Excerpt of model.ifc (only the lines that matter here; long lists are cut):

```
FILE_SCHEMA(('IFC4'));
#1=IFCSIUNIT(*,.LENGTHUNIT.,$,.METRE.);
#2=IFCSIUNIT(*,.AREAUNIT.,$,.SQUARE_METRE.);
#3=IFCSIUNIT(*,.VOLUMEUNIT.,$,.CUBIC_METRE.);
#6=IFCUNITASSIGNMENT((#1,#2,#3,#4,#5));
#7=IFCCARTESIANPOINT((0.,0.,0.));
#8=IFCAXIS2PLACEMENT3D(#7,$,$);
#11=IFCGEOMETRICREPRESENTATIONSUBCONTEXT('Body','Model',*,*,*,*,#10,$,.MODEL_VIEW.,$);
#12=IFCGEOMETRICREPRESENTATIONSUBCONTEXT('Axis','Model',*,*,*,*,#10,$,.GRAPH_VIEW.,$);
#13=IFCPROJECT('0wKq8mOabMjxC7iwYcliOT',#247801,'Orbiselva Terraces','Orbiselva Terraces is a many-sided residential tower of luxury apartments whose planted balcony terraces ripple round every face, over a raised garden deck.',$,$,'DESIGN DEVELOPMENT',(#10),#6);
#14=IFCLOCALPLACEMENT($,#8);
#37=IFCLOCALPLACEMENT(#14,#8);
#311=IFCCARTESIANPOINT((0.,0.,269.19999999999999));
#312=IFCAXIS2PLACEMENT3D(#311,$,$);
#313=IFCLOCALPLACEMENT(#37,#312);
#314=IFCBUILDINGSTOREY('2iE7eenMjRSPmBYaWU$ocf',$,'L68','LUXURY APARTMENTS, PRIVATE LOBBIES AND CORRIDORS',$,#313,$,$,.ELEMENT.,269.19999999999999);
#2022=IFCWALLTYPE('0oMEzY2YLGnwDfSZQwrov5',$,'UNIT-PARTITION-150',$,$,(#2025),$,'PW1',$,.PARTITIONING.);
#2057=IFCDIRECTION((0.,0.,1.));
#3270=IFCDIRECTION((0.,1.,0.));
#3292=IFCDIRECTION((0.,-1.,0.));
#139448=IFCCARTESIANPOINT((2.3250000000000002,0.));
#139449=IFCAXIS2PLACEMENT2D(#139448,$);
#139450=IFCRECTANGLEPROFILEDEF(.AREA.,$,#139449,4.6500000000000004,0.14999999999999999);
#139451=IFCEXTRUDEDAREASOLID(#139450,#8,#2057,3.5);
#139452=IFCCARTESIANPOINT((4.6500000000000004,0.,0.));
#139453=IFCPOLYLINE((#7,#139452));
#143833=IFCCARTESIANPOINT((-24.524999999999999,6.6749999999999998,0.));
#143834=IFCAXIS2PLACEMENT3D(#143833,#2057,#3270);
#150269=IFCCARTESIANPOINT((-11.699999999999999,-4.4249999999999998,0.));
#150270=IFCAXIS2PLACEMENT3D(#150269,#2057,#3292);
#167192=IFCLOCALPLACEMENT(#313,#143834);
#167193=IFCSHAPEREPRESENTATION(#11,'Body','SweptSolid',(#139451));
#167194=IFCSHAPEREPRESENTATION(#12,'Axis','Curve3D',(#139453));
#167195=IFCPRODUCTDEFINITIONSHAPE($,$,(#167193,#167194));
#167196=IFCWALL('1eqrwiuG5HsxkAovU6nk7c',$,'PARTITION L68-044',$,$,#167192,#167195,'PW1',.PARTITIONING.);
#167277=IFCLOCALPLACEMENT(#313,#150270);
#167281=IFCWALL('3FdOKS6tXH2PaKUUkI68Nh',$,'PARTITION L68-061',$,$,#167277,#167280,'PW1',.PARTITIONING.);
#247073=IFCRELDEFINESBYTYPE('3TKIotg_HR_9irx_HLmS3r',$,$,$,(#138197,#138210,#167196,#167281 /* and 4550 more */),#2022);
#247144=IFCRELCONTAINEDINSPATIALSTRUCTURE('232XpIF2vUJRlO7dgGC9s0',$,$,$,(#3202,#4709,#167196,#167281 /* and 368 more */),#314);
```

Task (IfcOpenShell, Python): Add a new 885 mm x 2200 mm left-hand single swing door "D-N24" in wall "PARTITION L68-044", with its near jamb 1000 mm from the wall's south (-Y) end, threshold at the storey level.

```python
import numpy as np
import ifcopenshell
import ifcopenshell.api.feature
import ifcopenshell.api.geometry
import ifcopenshell.api.root
import ifcopenshell.api.spatial
import ifcopenshell.geom
import ifcopenshell.util.element
import ifcopenshell.util.placement
import ifcopenshell.util.representation
import ifcopenshell.util.shape
import ifcopenshell.util.unit

model = ifcopenshell.open("model.ifc")
unit_scale = ifcopenshell.util.unit.calculate_unit_scale(model)
settings = ifcopenshell.geom.settings()


def volume(element):
    """Net volume in cubic metres, openings subtracted."""
    shape = ifcopenshell.geom.create_shape(settings, element)
    return ifcopenshell.util.shape.get_volume(shape.geometry)


wall = model.by_guid("1eqrwiuG5HsxkAovU6nk7c")
storey = ifcopenshell.util.element.get_container(wall, ifc_class="IfcBuildingStorey")
context = ifcopenshell.util.representation.get_context(model, "Model", "Body", "MODEL_VIEW")
before = volume(wall)

width, height, from_end, sill = 0.885, 2.2, 1, 0.0  # metres

# The wall runs along its own X axis, and the end named is its -X end.
wall_shape = ifcopenshell.geom.create_shape(settings, wall)
x, y, z = ifcopenshell.util.shape.get_vertices(wall_shape.geometry).T
start = x.min() + from_end
face, thickness = float(y.min()), float(y.max() - y.min())
wall_matrix = ifcopenshell.util.placement.get_local_placement(wall.ObjectPlacement)
level = ifcopenshell.util.placement.get_local_placement(storey.ObjectPlacement)[2, 3]


def in_wall(x, y):
    """Placement at x, y metres in the wall's axes, at sill height."""
    matrix = wall_matrix.copy()
    matrix[:, 3] = wall_matrix @ np.array([x / unit_scale, y / unit_scale, 0.0, 1.0])
    matrix[2, 3] = level + sill / unit_scale
    return matrix


# Opening: a box that overshoots both wall faces by 50 mm.
opening = ifcopenshell.api.root.create_entity(model, ifc_class="IfcOpeningElement", predefined_type="OPENING")
box = ifcopenshell.api.geometry.add_wall_representation(
    model, context=context, length=width, height=height, thickness=thickness + 0.1
)
ifcopenshell.api.geometry.assign_representation(model, product=opening, representation=box)
ifcopenshell.api.geometry.edit_object_placement(model, product=opening, matrix=in_wall(start, face - 0.05), is_si=False)
ifcopenshell.api.feature.add_feature(model, feature=opening, element=wall)

door = ifcopenshell.api.root.create_entity(model, ifc_class="IfcDoor", name="D-N24", predefined_type="DOOR")
door.OverallWidth, door.OverallHeight = width / unit_scale, height / unit_scale
door.OperationType = "SINGLE_SWING_LEFT"
body = ifcopenshell.api.geometry.add_door_representation(
    model,
    context=context,
    overall_width=door.OverallWidth,
    overall_height=door.OverallHeight,
    operation_type="SINGLE_SWING_LEFT",
    lining_properties={"LiningDepth": thickness / unit_scale, "ThresholdDepth": thickness / unit_scale},
)
ifcopenshell.api.geometry.assign_representation(model, product=door, representation=body)
ifcopenshell.api.spatial.assign_container(model, products=[door], relating_structure=storey)
ifcopenshell.api.feature.add_filling(model, opening=opening, element=door)

# The lining spans the wall, so the door starts at the wall face.
ifcopenshell.api.geometry.edit_object_placement(model, product=door, matrix=in_wall(start, face), is_si=False)

after = volume(wall)

print(f"wall volume {before:.3f} -> {after:.3f} m3")

model.write("model_v2.ifc")
```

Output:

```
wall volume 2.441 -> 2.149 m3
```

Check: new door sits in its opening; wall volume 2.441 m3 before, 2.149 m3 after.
